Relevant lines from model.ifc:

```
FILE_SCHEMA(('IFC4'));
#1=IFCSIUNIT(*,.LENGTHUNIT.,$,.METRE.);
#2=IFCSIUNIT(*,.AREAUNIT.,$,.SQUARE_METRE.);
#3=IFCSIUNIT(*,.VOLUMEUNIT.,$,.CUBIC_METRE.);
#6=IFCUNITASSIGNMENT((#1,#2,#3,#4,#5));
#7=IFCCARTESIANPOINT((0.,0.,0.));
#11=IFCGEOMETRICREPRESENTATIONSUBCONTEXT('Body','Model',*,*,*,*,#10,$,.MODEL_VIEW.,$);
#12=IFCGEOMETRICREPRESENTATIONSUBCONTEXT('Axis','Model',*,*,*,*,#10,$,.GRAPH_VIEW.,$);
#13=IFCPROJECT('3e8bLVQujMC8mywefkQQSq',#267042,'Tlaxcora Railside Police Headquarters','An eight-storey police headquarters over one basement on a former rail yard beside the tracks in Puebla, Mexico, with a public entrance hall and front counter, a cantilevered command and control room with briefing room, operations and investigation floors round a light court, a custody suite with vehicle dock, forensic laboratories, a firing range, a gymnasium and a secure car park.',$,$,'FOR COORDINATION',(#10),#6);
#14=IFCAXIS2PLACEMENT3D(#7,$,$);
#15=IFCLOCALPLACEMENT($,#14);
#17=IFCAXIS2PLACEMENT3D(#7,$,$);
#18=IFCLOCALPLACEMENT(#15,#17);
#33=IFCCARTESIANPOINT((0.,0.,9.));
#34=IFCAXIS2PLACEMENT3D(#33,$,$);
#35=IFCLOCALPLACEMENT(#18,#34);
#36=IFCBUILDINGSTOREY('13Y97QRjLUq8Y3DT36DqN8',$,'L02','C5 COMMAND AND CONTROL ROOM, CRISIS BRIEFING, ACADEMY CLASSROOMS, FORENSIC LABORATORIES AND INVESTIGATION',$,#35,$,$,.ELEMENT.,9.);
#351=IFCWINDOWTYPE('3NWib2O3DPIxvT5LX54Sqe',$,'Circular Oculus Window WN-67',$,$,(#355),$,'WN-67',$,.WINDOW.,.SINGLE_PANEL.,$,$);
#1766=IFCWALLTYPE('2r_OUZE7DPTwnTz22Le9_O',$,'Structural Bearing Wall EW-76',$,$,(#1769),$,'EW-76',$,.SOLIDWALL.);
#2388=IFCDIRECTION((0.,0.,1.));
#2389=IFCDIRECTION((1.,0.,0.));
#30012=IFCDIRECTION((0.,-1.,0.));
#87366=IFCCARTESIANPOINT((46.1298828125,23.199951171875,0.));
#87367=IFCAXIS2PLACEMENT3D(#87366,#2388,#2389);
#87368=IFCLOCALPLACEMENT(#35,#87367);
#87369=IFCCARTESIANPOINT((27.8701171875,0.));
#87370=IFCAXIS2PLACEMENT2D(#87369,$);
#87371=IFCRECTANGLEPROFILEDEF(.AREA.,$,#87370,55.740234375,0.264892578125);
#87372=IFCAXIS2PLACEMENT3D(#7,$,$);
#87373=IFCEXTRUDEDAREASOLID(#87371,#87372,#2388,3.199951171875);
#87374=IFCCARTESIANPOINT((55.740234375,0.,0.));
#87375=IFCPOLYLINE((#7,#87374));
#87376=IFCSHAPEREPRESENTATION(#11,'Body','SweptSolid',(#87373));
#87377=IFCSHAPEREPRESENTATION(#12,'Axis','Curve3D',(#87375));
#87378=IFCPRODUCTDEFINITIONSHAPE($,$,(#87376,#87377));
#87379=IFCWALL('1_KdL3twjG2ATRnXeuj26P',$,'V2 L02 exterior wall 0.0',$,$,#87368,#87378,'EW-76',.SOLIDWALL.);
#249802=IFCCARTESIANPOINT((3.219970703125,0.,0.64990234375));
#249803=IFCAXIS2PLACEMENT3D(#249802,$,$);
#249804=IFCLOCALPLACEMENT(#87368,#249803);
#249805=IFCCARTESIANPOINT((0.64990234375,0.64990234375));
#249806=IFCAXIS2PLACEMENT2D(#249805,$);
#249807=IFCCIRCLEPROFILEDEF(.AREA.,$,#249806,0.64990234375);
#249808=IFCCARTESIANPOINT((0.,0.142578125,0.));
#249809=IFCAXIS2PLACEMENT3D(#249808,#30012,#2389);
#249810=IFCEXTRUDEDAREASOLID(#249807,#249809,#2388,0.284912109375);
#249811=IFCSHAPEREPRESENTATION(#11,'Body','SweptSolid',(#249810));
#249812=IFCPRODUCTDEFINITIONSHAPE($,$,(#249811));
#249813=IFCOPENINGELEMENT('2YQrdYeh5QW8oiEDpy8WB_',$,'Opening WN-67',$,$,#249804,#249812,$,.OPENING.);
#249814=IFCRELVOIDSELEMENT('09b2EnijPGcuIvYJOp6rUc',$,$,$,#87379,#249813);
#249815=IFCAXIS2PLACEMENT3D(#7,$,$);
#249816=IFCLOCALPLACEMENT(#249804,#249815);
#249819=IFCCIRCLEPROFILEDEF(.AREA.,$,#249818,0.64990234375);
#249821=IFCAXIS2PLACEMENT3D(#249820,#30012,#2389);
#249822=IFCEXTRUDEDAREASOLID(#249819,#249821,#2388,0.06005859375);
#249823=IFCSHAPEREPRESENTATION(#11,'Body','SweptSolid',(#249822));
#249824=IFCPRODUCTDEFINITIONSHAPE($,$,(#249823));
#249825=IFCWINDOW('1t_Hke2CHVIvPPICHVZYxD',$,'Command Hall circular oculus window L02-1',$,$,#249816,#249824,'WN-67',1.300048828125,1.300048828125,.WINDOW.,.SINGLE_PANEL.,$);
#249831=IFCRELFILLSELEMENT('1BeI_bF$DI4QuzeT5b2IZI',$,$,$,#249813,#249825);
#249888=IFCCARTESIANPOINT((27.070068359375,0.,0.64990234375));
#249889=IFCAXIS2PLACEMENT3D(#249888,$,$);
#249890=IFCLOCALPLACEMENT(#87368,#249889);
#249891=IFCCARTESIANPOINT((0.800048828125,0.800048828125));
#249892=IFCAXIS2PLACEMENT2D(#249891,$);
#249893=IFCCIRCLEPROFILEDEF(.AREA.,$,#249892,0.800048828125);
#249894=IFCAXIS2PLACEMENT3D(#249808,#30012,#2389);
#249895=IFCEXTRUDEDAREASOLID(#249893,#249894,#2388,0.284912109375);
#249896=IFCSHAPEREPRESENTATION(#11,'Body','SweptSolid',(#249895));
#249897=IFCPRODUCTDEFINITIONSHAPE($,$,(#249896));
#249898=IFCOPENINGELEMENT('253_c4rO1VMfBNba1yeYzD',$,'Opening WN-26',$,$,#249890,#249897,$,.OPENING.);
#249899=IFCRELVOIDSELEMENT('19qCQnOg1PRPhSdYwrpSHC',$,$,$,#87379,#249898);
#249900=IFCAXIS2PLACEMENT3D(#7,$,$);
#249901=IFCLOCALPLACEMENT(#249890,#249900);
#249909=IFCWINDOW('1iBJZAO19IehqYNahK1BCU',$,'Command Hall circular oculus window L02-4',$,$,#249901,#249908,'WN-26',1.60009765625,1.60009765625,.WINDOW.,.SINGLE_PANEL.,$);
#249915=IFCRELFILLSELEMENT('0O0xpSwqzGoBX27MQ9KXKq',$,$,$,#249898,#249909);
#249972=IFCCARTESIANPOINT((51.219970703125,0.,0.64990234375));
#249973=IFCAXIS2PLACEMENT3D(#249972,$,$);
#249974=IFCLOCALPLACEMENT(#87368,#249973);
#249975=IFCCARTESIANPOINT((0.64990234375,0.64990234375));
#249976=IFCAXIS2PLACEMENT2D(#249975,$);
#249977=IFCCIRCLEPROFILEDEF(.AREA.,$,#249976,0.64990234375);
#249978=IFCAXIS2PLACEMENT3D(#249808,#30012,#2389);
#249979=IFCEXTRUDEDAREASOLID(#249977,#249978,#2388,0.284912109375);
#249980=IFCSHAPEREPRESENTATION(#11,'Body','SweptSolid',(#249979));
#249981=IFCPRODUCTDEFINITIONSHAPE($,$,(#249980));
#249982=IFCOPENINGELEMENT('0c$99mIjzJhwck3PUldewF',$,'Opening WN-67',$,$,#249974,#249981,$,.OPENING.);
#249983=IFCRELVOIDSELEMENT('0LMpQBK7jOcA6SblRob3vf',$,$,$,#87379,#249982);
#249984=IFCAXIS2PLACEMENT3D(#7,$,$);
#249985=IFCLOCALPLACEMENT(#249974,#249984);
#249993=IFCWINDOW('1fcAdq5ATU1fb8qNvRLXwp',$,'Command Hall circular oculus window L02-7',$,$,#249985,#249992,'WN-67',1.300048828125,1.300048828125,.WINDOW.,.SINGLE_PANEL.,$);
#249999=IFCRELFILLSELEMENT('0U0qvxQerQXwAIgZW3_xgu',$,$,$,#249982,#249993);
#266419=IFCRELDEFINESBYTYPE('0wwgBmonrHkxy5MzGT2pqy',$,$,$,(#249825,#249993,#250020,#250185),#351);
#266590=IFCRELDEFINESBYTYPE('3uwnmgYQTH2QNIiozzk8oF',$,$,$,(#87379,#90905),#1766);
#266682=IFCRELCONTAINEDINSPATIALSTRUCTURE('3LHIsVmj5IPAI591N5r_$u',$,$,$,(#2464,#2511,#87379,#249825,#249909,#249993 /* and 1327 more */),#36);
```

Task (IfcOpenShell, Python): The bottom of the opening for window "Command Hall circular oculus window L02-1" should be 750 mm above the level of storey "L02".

```python
import numpy as np
import ifcopenshell
import ifcopenshell.api.geometry
import ifcopenshell.geom
import ifcopenshell.util.element
import ifcopenshell.util.placement
import ifcopenshell.util.shape
import ifcopenshell.util.unit

model = ifcopenshell.open("model.ifc")
unit_scale = ifcopenshell.util.unit.calculate_unit_scale(model)

window = model.by_id(249825)
opening = window.FillsVoids[0].RelatingOpeningElement
storey = ifcopenshell.util.element.get_container(window, ifc_class="IfcBuildingStorey")
level = ifcopenshell.util.placement.get_local_placement(storey.ObjectPlacement)[2, 3]

# The opening's origin need not be at the sill, so measure its lowest point.
shape = ifcopenshell.geom.create_shape(ifcopenshell.geom.settings(), opening)
bottom = ifcopenshell.util.shape.get_shape_bottom_elevation(shape, shape.geometry) / unit_scale
dz = level + 0.75 / unit_scale - bottom

shift = np.array([0.0, 0.0, dz])
# The window is placed relative to its opening, so it follows when the opening moves.
matrix = ifcopenshell.util.placement.get_local_placement(opening.ObjectPlacement)
matrix[:3, 3] += shift
ifcopenshell.api.geometry.edit_object_placement(
    model, product=opening, matrix=matrix, is_si=False, should_transform_children=True
)

print(f"moved by {dz * unit_scale:+.3f} m")

model.write("model-out.ifc")
```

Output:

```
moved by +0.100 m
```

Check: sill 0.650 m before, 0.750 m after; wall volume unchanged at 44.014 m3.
